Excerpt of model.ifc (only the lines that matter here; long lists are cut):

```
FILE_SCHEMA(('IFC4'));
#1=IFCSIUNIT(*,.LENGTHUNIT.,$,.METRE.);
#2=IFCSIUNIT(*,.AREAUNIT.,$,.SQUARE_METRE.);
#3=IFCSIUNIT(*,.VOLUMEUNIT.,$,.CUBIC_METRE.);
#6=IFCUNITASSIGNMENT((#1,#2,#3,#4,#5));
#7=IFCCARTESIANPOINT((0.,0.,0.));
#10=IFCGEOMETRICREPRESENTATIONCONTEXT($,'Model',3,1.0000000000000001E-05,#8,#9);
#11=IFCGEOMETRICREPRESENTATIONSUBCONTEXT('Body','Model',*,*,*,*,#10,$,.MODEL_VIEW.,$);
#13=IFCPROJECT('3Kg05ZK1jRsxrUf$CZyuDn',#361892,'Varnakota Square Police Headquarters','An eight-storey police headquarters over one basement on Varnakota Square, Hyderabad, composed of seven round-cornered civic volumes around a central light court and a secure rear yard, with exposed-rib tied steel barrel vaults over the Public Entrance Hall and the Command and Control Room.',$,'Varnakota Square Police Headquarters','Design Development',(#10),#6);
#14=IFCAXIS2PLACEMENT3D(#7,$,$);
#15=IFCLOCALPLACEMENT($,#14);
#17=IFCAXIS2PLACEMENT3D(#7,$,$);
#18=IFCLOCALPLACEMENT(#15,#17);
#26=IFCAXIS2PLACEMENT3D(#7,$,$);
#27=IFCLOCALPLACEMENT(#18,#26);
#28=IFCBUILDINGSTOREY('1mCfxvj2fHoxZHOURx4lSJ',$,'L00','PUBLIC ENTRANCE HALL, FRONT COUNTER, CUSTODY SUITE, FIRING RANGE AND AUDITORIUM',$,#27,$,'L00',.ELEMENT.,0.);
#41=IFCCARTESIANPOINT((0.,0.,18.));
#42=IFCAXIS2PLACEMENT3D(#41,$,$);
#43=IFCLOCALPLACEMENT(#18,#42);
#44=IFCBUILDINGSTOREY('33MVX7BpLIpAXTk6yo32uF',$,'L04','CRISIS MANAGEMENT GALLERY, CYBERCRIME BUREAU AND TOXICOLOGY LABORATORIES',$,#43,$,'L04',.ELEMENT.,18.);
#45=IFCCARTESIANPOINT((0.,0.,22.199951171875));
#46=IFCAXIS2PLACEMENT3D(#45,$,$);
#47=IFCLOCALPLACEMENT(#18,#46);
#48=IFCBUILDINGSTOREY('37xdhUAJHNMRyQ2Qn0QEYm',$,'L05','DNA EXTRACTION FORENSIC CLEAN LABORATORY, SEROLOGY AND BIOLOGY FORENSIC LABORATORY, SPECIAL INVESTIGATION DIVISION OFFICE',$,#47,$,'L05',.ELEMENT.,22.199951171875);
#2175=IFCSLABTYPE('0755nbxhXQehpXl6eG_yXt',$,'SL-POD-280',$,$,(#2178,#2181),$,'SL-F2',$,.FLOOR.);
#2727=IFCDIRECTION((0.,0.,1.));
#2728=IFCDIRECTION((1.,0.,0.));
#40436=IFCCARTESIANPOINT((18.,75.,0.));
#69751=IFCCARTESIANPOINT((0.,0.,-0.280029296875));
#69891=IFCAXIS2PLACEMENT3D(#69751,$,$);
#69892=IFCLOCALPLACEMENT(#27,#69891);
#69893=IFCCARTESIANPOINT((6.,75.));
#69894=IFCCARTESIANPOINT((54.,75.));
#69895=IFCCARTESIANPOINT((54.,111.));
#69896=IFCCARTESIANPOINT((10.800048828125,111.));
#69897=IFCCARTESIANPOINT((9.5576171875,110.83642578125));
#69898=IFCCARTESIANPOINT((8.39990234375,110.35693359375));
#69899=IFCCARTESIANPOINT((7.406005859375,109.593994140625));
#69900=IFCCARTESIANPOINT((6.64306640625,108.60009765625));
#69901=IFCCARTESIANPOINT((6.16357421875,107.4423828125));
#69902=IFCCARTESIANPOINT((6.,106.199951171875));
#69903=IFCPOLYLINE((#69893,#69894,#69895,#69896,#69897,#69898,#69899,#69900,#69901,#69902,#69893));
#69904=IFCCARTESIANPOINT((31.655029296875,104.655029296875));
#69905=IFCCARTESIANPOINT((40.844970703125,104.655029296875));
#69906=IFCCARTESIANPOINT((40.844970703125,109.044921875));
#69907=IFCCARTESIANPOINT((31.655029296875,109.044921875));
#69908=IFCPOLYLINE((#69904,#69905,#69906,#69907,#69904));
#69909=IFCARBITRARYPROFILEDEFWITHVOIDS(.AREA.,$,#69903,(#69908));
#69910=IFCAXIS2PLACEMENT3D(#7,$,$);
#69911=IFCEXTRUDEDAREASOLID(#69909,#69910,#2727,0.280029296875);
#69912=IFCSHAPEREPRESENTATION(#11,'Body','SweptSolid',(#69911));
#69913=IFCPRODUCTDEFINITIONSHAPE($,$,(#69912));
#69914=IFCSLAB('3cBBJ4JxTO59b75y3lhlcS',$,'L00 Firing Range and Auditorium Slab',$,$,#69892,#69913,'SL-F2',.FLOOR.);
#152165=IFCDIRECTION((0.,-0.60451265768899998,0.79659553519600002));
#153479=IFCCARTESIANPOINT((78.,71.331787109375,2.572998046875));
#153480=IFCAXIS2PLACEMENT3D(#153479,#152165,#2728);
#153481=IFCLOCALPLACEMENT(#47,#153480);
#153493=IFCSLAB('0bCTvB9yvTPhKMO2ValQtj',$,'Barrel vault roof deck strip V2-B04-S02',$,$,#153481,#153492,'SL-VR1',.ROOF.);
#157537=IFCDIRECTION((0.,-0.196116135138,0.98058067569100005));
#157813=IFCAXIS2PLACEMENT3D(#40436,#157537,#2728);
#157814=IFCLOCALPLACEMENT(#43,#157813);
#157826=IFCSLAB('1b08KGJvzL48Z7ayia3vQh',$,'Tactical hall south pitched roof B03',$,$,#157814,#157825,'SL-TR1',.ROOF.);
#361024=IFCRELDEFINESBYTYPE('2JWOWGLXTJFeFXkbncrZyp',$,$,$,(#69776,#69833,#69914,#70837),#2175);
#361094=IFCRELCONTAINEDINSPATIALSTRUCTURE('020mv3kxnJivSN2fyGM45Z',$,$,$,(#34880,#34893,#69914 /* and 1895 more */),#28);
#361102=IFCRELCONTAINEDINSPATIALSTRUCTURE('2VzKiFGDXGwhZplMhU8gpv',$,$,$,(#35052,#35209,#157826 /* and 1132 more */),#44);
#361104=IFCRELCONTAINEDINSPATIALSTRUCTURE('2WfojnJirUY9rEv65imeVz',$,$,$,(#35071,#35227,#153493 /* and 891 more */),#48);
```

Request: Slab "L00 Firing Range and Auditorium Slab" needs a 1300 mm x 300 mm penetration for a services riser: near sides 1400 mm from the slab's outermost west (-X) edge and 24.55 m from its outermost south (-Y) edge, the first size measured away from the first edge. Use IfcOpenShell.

```python
import numpy as np
import ifcopenshell
import ifcopenshell.api.feature
import ifcopenshell.api.geometry
import ifcopenshell.api.root
import ifcopenshell.geom
import ifcopenshell.util.placement
import ifcopenshell.util.representation
import ifcopenshell.util.shape
import ifcopenshell.util.unit

model = ifcopenshell.open("model.ifc")
unit_scale = ifcopenshell.util.unit.calculate_unit_scale(model)
settings = ifcopenshell.geom.settings()


def volume(element):
    """Net volume in cubic metres, openings subtracted."""
    shape = ifcopenshell.geom.create_shape(settings, element)
    return ifcopenshell.util.shape.get_volume(shape.geometry)


slab = model.by_id(69914)
before = volume(slab)

# Extent in the slab's own axes, in metres. The edges named are its -X and -Y sides.
slab_shape = ifcopenshell.geom.create_shape(settings, slab)
vertices = ifcopenshell.util.shape.get_vertices(slab_shape.geometry)
x_min, y_min, bottom = vertices.min(axis=0)
top = vertices[:, 2].max()

opening = ifcopenshell.api.root.create_entity(model, ifc_class="IfcOpeningElement", name="Services riser opening", predefined_type="OPENING")
context = ifcopenshell.util.representation.get_context(model, "Model", "Body", "MODEL_VIEW")
width, depth = 1.3, 0.3
outline = [(0.0, 0.0), (width, 0.0), (width, depth), (0.0, depth), (0.0, 0.0)]
# Overshoot both faces by 50 mm so the cut is clean.
shape = ifcopenshell.api.geometry.add_slab_representation(
    model, context=context, depth=top - bottom + 0.1, polyline=outline
)
ifcopenshell.api.geometry.assign_representation(model, product=opening, representation=shape)

matrix = ifcopenshell.util.placement.get_local_placement(slab.ObjectPlacement)
matrix[:, 3] = matrix @ np.append(np.array([x_min + 1.4, y_min + 24.55, bottom - 0.05]) / unit_scale, 1.0)
ifcopenshell.api.geometry.edit_object_placement(model, product=opening, matrix=matrix, is_si=False)
ifcopenshell.api.feature.add_feature(model, feature=opening, element=slab)

after = volume(slab)

print(f"slab volume {before:.3f} -> {after:.3f} m3")

model.write("model_v2.ifc")
```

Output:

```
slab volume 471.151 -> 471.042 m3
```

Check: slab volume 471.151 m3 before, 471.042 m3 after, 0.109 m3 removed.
